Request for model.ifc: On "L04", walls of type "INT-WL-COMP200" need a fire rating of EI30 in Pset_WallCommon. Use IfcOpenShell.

First a look at what the model holds.

```python
import ifcopenshell
import ifcopenshell.util.element

model = ifcopenshell.open("model.ifc")
print(model.schema)
storey = next(s for s in model.by_type("IfcBuildingStorey") if s.Name == "L04")
walls = [e for e in ifcopenshell.util.element.get_decomposition(storey) if e.is_a("IfcWall")]
seen = {}
for e in walls:
    element_type = ifcopenshell.util.element.get_type(e)
    key = (element_type.Name if element_type != e and element_type else None, ifcopenshell.util.element.get_pset(e, "Pset_WallCommon", "FireRating"))
    seen[key] = seen.get(key, 0) + 1
for (name, value), count in sorted(seen.items(), key=str):
    print(count, "x", name, "|", value)
```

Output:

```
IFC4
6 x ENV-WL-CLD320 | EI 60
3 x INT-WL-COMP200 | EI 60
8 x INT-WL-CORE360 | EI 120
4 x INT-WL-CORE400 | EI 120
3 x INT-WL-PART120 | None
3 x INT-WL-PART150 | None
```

```python
import ifcopenshell
import ifcopenshell.api.pset
import ifcopenshell.util.element

model = ifcopenshell.open("model.ifc")

storey = next(s for s in model.by_type("IfcBuildingStorey") if s.Name == "L04")
walls = [e for e in ifcopenshell.util.element.get_decomposition(storey) if e.is_a("IfcWall")]

count = 0
for e in walls:
    element_type = ifcopenshell.util.element.get_type(e)
    if element_type in (None, e) or element_type.Name != "INT-WL-COMP200":
        continue
    # add_pset returns the element's existing set when there is one.
    pset = ifcopenshell.api.pset.add_pset(model, product=e, name="Pset_WallCommon")
    ifcopenshell.api.pset.edit_pset(model, pset=pset, properties={"FireRating": "EI30"})
    count += 1

print(count, "walls updated")

model.write("model_edited.ifc")
```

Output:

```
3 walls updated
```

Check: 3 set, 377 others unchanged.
